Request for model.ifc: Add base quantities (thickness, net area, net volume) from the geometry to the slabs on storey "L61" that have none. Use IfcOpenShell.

First a look at what the model holds.

```python
import ifcopenshell
import ifcopenshell.util.element
import ifcopenshell.util.unit

model = ifcopenshell.open("model.ifc")
print(model.schema)
for unit_type in ("LENGTHUNIT", "AREAUNIT", "VOLUMEUNIT"):
    print(unit_type, ifcopenshell.util.unit.calculate_unit_scale(model, unit_type))
storey = next(s for s in model.by_type("IfcBuildingStorey") if s.Name == "L61")
slabs = [e for e in ifcopenshell.util.element.get_decomposition(storey) if e.is_a("IfcSlab")]
for e in sorted(slabs, key=lambda e: e.id()):
    print(e.id(), e.is_a(), e.Name, list(ifcopenshell.util.element.get_psets(e, qtos_only=True)), sep=" | ")
```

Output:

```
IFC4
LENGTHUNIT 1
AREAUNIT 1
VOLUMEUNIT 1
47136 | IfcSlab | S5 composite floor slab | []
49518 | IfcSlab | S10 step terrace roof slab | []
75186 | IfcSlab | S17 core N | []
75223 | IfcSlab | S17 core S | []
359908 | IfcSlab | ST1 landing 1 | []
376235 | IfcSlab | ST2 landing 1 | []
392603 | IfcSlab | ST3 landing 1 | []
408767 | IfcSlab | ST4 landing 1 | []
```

```python
import ifcopenshell
import ifcopenshell.api.pset
import ifcopenshell.geom
import ifcopenshell.util.element
import ifcopenshell.util.shape
import ifcopenshell.util.unit

model = ifcopenshell.open("model.ifc")
unit_scale = ifcopenshell.util.unit.calculate_unit_scale(model)
area_scale = ifcopenshell.util.unit.calculate_unit_scale(model, "AREAUNIT")
volume_scale = ifcopenshell.util.unit.calculate_unit_scale(model, "VOLUMEUNIT")
settings = ifcopenshell.geom.settings()

storey = next(s for s in model.by_type("IfcBuildingStorey") if s.Name == "L61")
slabs = [e for e in ifcopenshell.util.element.get_decomposition(storey) if e.is_a("IfcSlab")]

for e in sorted(slabs, key=lambda e: e.id()):
    if ifcopenshell.util.element.get_psets(e, qtos_only=True, should_inherit=False):
        continue
    # Geometry comes back in metres, in the element's own axes.
    shape = ifcopenshell.geom.create_shape(settings, e)
    values = {
        "Width": ifcopenshell.util.shape.get_z(shape.geometry) / unit_scale,
        "NetArea": ifcopenshell.util.shape.get_footprint_area(shape.geometry) / area_scale,
        "NetVolume": ifcopenshell.util.shape.get_volume(shape.geometry) / volume_scale,
    }
    qto = ifcopenshell.api.pset.add_qto(model, product=e, name="Qto_SlabBaseQuantities")
    ifcopenshell.api.pset.edit_qto(model, qto=qto, properties=values)
    print(e.id(), {k: round(v, 3) for k, v in values.items()})

model.write("model_updated.ifc")
```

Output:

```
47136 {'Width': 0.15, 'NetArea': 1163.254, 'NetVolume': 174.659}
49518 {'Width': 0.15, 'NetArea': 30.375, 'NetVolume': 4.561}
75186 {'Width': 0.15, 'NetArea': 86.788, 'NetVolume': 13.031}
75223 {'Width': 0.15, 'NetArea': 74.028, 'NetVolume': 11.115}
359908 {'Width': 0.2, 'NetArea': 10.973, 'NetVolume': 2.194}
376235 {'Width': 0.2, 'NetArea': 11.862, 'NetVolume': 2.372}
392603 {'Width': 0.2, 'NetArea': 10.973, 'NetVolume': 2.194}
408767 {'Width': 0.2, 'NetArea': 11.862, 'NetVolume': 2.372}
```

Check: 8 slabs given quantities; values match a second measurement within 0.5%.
